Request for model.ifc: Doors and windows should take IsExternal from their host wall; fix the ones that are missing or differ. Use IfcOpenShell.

First a look at what the model holds.

```python
import ifcopenshell
import ifcopenshell.util.element

model = ifcopenshell.open("model.ifc")
print(model.schema)
seen = {}
for e in model.by_type("IfcDoor") + model.by_type("IfcWindow"):
    if not e.FillsVoids:
        continue
    host = e.FillsVoids[0].RelatingOpeningElement.VoidsElements[0].RelatingBuildingElement
    own = ifcopenshell.util.element.get_pset(e, f"Pset_{e.is_a()[3:].removesuffix('StandardCase')}Common", "IsExternal")
    wall = ifcopenshell.util.element.get_pset(host, "Pset_WallCommon", "IsExternal")
    seen[e.is_a(), own, wall] = seen.get((e.is_a(), own, wall), 0) + 1
for (cls, own, wall), count in sorted(seen.items(), key=str):
    print(count, cls, "IsExternal:", own, "| host wall:", wall)
```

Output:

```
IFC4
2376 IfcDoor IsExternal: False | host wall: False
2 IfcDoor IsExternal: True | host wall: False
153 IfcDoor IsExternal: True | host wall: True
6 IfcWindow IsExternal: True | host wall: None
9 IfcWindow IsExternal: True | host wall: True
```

```python
import ifcopenshell
import ifcopenshell.api.pset
import ifcopenshell.util.element

model = ifcopenshell.open("model.ifc")

count = 0
for ifc_class, pset_name in (("IfcDoor", "Pset_DoorCommon"), ("IfcWindow", "Pset_WindowCommon")):
    for e in model.by_type(ifc_class):
        if not e.FillsVoids:
            continue
        host = e.FillsVoids[0].RelatingOpeningElement.VoidsElements[0].RelatingBuildingElement
        external = ifcopenshell.util.element.get_pset(host, "Pset_WallCommon", "IsExternal")
        if external is None or ifcopenshell.util.element.get_pset(e, pset_name, "IsExternal") == external:
            continue
        found = ifcopenshell.util.element.get_pset(e, pset_name, should_inherit=False)
        if found:
            pset = model.by_id(found["id"])
            if len(ifcopenshell.util.element.get_elements_by_pset(pset)) > 1:
                pset = ifcopenshell.api.pset.unshare_pset(model, products=[e], pset=pset)[0]
        else:
            pset = ifcopenshell.api.pset.add_pset(model, product=e, name=pset_name)
        ifcopenshell.api.pset.edit_pset(model, pset=pset, properties={"IsExternal": external})
        count += 1

print(count, "updated")

model.write("model_rev.ifc")
```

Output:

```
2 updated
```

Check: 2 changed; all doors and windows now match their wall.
